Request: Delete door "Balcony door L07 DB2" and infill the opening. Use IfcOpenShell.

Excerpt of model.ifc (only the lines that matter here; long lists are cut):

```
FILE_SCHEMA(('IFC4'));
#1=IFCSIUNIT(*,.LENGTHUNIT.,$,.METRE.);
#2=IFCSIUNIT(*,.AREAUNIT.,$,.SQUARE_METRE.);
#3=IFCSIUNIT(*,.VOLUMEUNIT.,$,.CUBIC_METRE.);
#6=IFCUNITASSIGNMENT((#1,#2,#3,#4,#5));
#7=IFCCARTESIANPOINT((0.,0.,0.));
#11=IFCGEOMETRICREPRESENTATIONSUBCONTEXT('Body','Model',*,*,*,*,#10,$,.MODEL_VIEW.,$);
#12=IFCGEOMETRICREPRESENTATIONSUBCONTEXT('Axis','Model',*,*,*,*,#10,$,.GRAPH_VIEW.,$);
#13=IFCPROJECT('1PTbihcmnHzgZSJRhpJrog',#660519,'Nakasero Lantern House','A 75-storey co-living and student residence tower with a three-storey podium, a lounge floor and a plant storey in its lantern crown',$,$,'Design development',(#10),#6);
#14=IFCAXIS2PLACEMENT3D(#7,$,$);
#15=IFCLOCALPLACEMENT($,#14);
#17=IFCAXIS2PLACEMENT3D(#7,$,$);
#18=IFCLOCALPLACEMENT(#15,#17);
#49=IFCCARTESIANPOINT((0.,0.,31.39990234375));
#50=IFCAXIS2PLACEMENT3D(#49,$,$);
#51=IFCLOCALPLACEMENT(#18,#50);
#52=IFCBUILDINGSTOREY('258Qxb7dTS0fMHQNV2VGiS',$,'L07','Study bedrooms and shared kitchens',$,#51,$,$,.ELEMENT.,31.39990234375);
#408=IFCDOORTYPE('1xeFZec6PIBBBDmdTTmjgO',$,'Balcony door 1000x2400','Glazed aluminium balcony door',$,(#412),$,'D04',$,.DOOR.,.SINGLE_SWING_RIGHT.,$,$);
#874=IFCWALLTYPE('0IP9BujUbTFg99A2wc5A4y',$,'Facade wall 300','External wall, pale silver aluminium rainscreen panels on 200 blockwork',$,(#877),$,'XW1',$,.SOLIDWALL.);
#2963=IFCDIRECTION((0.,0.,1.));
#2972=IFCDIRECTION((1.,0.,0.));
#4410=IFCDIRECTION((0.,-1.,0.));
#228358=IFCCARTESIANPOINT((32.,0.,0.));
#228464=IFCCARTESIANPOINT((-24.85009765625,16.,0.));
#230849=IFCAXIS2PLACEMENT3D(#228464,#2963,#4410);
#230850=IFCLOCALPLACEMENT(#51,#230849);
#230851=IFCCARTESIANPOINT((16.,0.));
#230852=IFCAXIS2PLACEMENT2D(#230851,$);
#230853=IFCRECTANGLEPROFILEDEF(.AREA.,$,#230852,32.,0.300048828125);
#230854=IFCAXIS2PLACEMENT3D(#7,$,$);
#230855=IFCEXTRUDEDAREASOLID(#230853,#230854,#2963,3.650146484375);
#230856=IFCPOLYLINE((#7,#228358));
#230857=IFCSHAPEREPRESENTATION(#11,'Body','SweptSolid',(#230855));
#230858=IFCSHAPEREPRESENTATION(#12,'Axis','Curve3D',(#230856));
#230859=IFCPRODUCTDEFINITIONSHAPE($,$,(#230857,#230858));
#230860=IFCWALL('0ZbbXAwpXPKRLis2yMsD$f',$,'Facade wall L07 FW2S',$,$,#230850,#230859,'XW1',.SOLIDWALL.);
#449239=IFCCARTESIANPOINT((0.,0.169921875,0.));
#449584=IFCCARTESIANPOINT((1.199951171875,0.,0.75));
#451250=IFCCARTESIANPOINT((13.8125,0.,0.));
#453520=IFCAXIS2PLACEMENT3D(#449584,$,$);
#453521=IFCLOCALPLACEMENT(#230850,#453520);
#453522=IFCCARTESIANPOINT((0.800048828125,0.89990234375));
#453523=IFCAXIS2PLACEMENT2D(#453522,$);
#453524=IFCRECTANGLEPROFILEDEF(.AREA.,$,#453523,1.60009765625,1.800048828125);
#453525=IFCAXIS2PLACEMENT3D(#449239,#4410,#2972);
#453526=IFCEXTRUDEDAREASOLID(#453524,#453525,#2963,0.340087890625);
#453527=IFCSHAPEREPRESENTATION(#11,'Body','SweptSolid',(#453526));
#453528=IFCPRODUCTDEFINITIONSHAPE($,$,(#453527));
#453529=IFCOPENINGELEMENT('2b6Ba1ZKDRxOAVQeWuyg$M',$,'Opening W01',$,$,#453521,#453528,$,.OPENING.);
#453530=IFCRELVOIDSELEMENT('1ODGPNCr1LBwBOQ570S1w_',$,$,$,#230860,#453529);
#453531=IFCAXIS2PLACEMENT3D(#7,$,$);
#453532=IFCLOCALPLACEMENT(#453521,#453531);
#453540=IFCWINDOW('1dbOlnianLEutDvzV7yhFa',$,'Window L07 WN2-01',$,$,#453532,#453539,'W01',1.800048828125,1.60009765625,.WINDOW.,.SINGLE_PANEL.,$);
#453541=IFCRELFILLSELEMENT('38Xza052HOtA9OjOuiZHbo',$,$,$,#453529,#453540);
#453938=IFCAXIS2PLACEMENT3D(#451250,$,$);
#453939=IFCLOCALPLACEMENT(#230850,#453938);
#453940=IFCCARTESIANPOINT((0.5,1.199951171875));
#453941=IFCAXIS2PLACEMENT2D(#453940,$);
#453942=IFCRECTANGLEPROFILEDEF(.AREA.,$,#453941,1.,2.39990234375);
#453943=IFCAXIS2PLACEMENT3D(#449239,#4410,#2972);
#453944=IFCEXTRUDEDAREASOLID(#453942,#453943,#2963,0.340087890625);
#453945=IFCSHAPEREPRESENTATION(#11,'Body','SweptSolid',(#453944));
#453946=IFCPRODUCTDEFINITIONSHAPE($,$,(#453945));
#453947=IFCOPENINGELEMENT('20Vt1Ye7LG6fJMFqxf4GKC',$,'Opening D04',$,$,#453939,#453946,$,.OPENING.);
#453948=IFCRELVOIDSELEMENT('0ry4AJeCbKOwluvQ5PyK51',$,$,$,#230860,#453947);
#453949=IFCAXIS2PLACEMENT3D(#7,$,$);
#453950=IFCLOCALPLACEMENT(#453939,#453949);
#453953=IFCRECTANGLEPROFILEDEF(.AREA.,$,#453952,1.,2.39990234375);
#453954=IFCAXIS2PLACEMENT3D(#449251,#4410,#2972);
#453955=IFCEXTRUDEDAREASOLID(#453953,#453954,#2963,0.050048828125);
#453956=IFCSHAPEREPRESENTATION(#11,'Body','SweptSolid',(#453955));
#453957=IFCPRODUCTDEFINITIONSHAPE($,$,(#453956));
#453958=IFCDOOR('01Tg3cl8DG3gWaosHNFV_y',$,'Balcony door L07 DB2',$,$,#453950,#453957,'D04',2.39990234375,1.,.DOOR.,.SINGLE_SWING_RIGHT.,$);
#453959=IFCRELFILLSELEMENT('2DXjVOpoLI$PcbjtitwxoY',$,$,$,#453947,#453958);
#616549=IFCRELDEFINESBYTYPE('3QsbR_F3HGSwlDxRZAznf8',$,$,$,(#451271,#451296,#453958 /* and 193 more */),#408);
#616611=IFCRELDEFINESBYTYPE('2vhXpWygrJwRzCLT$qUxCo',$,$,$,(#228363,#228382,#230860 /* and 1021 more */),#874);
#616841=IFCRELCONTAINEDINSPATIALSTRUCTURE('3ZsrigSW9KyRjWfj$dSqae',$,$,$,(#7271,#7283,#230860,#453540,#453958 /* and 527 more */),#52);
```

```python
import ifcopenshell
import ifcopenshell.api.feature
import ifcopenshell.api.root
import ifcopenshell.geom
import ifcopenshell.util.shape

model = ifcopenshell.open("model.ifc")
settings = ifcopenshell.geom.settings()


def volume(element):
    """Net volume in cubic metres, openings subtracted."""
    shape = ifcopenshell.geom.create_shape(settings, element)
    return ifcopenshell.util.shape.get_volume(shape.geometry)


door = model.by_id(453958)
opening = door.FillsVoids[0].RelatingOpeningElement
wall = opening.VoidsElements[0].RelatingBuildingElement
before = volume(wall)

ifcopenshell.api.root.remove_product(model, product=door)
ifcopenshell.api.feature.remove_feature(model, feature=opening)

after = volume(wall)

print(f"wall volume {before:.3f} -> {after:.3f} m3")

model.write("model_v2.ifc")
```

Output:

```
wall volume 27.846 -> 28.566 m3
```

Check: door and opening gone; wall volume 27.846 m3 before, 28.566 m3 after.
